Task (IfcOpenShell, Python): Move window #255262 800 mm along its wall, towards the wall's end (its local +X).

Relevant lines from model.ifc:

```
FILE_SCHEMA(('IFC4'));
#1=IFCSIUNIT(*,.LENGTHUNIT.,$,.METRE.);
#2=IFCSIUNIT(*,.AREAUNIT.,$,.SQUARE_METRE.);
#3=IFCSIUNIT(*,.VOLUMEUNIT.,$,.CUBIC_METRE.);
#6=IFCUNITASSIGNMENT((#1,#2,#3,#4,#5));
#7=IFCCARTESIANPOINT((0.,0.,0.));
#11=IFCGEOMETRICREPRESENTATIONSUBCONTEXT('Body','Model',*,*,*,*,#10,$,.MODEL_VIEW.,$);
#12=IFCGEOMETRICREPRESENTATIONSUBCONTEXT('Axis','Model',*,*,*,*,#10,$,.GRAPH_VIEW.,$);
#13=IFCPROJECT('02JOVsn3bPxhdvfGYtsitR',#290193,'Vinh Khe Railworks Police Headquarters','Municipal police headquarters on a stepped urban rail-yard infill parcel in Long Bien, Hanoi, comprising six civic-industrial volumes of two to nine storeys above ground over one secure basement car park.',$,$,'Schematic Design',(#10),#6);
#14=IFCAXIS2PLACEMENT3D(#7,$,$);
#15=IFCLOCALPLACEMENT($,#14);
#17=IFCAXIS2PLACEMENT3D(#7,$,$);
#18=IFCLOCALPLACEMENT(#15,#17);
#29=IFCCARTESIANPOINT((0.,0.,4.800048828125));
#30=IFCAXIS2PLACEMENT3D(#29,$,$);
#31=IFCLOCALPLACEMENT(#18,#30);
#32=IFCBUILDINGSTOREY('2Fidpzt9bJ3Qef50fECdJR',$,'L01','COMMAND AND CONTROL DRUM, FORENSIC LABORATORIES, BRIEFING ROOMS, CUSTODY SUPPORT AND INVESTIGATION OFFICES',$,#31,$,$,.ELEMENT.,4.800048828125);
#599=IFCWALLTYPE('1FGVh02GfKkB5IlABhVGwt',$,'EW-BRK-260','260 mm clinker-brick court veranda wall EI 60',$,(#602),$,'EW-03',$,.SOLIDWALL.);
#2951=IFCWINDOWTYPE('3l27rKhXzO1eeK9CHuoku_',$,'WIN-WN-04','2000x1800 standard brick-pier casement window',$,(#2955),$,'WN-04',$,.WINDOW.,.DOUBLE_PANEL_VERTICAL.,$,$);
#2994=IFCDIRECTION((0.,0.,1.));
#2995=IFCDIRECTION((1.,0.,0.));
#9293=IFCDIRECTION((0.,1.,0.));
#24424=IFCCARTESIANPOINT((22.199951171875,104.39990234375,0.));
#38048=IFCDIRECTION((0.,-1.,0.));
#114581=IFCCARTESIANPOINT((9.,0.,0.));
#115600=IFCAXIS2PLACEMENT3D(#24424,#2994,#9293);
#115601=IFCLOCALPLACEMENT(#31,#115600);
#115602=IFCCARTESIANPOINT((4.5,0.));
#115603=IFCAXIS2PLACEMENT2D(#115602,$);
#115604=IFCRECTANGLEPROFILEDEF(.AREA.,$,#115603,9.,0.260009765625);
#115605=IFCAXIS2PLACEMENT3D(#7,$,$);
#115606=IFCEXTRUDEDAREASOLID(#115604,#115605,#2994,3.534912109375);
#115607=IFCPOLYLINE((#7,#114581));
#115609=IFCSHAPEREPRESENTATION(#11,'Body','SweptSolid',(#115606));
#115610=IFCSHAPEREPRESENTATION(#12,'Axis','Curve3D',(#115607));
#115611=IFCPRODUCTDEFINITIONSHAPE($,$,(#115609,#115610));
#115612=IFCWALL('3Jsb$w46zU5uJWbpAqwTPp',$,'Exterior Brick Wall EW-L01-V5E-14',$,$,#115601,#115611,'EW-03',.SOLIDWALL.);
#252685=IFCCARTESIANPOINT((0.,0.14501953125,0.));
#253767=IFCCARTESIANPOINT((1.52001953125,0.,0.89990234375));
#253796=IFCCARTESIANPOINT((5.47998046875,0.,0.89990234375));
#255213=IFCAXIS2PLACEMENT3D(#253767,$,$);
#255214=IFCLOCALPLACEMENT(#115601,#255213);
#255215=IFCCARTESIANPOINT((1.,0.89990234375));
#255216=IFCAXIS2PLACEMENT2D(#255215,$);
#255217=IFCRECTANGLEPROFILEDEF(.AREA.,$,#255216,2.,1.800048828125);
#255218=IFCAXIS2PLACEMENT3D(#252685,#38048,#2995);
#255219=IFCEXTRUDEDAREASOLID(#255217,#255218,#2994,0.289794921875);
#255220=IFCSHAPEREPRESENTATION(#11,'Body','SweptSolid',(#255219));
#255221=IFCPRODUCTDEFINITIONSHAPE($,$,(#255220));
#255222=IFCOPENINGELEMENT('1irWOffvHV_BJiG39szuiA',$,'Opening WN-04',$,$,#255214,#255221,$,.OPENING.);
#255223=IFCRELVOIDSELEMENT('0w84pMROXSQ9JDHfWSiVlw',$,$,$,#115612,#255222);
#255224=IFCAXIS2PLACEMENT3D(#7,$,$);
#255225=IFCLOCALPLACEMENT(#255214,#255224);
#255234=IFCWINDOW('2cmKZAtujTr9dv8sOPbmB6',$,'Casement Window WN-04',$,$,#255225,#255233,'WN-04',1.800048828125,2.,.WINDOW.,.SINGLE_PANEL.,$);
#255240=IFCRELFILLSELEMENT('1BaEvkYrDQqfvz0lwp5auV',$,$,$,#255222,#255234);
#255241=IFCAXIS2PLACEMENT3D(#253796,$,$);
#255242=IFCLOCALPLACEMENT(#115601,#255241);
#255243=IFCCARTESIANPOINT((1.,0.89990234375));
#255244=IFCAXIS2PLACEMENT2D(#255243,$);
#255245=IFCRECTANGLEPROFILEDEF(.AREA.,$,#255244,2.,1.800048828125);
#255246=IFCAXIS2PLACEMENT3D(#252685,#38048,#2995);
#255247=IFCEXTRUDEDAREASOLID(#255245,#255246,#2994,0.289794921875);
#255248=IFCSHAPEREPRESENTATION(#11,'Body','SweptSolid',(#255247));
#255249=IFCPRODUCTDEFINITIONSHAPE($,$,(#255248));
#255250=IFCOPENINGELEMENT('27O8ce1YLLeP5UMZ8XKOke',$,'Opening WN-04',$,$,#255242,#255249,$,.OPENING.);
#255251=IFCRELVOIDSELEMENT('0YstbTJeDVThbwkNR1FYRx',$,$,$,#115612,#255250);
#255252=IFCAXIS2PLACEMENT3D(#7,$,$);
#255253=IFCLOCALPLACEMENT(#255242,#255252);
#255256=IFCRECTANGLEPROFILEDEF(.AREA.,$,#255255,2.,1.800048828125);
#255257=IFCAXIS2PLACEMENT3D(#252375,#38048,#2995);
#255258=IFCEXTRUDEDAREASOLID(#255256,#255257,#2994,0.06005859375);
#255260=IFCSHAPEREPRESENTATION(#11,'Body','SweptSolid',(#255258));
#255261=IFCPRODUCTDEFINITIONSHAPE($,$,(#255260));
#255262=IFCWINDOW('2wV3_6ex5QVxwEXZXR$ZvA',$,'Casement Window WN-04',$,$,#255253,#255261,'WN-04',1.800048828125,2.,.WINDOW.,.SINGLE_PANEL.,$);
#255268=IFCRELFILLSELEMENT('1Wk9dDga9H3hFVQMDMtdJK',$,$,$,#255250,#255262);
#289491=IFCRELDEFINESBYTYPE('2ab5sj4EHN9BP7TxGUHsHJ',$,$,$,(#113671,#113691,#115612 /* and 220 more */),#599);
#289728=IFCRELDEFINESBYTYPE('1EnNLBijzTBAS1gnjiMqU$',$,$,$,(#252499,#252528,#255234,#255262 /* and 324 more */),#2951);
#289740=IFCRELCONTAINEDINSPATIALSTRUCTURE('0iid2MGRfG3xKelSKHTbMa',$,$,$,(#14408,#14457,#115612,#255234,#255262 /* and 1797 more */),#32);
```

```python
import ifcopenshell
import ifcopenshell.api.geometry
import ifcopenshell.util.placement

model = ifcopenshell.open("model.ifc")

window = model.by_guid("2wV3_6ex5QVxwEXZXR$ZvA")
opening = window.FillsVoids[0].RelatingOpeningElement
wall = opening.VoidsElements[0].RelatingBuildingElement

wall_matrix = ifcopenshell.util.placement.get_local_placement(wall.ObjectPlacement)
shift = wall_matrix[:3, 0] * 0.8
before = ifcopenshell.util.placement.get_local_placement(window.ObjectPlacement)[:3, 3].copy()

# The window is placed relative to its opening, so it follows when the opening moves.
matrix = ifcopenshell.util.placement.get_local_placement(opening.ObjectPlacement)
matrix[:3, 3] += shift
ifcopenshell.api.geometry.edit_object_placement(
    model, product=opening, matrix=matrix, is_si=False, should_transform_children=True
)

after = ifcopenshell.util.placement.get_local_placement(window.ObjectPlacement)[:3, 3]
print("window moved by", (after - before).round(3) + 0.0)

model.write("model_rev.ifc")
```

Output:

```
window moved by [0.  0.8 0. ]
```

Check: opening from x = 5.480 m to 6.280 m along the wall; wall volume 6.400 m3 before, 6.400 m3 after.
